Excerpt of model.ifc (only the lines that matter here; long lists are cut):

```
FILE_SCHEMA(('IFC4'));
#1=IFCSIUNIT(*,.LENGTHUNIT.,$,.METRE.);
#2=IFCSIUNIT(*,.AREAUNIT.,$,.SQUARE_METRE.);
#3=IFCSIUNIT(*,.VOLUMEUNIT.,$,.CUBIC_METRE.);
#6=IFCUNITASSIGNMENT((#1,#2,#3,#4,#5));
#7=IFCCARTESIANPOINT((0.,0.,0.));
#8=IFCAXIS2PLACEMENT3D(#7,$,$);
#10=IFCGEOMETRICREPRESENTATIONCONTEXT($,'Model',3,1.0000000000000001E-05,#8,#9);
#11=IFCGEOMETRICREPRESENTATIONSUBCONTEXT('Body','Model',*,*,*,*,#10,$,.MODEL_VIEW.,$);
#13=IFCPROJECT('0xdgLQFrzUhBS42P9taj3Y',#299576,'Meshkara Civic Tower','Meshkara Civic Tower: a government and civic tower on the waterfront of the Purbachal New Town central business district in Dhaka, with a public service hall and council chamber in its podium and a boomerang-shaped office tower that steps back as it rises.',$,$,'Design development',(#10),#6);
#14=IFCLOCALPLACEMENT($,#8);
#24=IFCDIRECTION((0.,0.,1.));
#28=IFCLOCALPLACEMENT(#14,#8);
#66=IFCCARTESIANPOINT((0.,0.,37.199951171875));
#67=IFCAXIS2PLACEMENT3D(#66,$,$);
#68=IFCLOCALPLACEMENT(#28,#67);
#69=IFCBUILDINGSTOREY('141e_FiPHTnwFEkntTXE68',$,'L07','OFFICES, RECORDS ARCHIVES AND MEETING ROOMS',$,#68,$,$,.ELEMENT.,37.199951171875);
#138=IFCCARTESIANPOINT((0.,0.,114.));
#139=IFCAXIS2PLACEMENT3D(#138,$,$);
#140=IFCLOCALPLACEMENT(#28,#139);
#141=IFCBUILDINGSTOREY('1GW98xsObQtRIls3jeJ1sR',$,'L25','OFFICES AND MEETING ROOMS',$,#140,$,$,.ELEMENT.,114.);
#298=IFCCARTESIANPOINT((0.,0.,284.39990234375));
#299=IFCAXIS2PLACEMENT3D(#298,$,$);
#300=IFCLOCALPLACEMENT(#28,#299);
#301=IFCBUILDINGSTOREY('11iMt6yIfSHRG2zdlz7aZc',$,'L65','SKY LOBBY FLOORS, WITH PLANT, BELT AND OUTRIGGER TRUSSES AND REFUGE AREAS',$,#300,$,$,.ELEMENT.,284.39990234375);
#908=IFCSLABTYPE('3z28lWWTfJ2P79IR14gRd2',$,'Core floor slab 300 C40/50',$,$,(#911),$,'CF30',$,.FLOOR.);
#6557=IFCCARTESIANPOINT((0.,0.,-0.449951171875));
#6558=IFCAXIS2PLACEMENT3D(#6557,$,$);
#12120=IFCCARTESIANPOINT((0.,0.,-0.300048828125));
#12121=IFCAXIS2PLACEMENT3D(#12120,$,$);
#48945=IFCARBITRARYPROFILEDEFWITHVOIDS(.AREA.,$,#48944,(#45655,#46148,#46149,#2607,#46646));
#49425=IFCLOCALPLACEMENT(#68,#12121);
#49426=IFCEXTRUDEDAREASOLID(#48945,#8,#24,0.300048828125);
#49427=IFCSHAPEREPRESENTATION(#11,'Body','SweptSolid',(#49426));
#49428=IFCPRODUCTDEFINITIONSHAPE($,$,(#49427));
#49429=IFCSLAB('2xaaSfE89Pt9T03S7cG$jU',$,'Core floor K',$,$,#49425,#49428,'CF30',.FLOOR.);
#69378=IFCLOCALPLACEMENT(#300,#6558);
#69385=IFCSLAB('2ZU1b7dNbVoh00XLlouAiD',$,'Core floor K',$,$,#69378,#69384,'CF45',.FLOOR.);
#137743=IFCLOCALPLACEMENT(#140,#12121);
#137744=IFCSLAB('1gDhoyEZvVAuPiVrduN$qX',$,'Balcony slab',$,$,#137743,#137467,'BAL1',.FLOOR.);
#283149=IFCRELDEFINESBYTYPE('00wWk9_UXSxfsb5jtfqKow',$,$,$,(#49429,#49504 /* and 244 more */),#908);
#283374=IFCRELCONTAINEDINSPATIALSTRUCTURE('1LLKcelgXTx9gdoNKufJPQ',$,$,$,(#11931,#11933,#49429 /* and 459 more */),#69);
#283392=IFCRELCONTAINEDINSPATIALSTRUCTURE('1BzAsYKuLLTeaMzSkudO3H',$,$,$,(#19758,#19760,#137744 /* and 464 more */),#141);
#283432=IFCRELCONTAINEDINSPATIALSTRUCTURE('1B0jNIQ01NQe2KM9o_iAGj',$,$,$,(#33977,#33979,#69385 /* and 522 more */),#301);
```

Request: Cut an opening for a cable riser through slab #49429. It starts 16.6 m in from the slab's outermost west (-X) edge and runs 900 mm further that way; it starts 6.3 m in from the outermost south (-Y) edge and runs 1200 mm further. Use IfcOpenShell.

```python
import numpy as np
import ifcopenshell
import ifcopenshell.api.feature
import ifcopenshell.api.geometry
import ifcopenshell.api.root
import ifcopenshell.geom
import ifcopenshell.util.placement
import ifcopenshell.util.representation
import ifcopenshell.util.shape
import ifcopenshell.util.unit

model = ifcopenshell.open("model.ifc")
unit_scale = ifcopenshell.util.unit.calculate_unit_scale(model)
settings = ifcopenshell.geom.settings()


def volume(element):
    """Net volume in cubic metres, openings subtracted."""
    shape = ifcopenshell.geom.create_shape(settings, element)
    return ifcopenshell.util.shape.get_volume(shape.geometry)


slab = model.by_guid("2xaaSfE89Pt9T03S7cG$jU")
before = volume(slab)

# Extent in the slab's own axes, in metres. The edges named are its -X and -Y sides.
slab_shape = ifcopenshell.geom.create_shape(settings, slab)
vertices = ifcopenshell.util.shape.get_vertices(slab_shape.geometry)
x_min, y_min, bottom = vertices.min(axis=0)
top = vertices[:, 2].max()

opening = ifcopenshell.api.root.create_entity(model, ifc_class="IfcOpeningElement", name="Cable riser opening", predefined_type="OPENING")
context = ifcopenshell.util.representation.get_context(model, "Model", "Body", "MODEL_VIEW")
width, depth = 0.9, 1.2
outline = [(0.0, 0.0), (width, 0.0), (width, depth), (0.0, depth), (0.0, 0.0)]
# Overshoot both faces by 50 mm so the cut is clean.
shape = ifcopenshell.api.geometry.add_slab_representation(
    model, context=context, depth=top - bottom + 0.1, polyline=outline
)
ifcopenshell.api.geometry.assign_representation(model, product=opening, representation=shape)

matrix = ifcopenshell.util.placement.get_local_placement(slab.ObjectPlacement)
matrix[:, 3] = matrix @ np.append(np.array([x_min + 16.6, y_min + 6.3, bottom - 0.05]) / unit_scale, 1.0)
ifcopenshell.api.geometry.edit_object_placement(model, product=opening, matrix=matrix, is_si=False)
ifcopenshell.api.feature.add_feature(model, feature=opening, element=slab)

after = volume(slab)

print(f"slab volume {before:.3f} -> {after:.3f} m3")

model.write("model_edited.ifc")
```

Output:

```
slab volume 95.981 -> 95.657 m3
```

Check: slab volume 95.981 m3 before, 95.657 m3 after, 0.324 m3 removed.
